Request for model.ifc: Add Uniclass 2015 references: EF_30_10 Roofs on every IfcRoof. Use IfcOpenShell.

First a look at what the model holds.

```python
import ifcopenshell

model = ifcopenshell.open("model.ifc")
print(model.schema)
print("classifications:", [c.Name for c in model.by_type("IfcClassification")])
for ifc_class in ("IfcDoor", "IfcRoof", "IfcStair", "IfcWall", "IfcWindow"):
    print(ifc_class, len(model.by_type(ifc_class)))
```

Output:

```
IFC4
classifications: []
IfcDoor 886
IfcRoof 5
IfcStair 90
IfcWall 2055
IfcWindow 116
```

```python
import ifcopenshell
import ifcopenshell.api.classification

model = ifcopenshell.open("model.ifc")

system = ifcopenshell.api.classification.add_classification(model, classification="Uniclass 2015")

codes = {
    "IfcRoof": ("EF_30_10", "Roofs"),
}
for ifc_class, (code, name) in codes.items():
    products = model.by_type(ifc_class)
    ifcopenshell.api.classification.add_reference(
        model, products=products, classification=system, identification=code, name=name
    )
    print(code, len(products))

model.write("model_v2.ifc")
```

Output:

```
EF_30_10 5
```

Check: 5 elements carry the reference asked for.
